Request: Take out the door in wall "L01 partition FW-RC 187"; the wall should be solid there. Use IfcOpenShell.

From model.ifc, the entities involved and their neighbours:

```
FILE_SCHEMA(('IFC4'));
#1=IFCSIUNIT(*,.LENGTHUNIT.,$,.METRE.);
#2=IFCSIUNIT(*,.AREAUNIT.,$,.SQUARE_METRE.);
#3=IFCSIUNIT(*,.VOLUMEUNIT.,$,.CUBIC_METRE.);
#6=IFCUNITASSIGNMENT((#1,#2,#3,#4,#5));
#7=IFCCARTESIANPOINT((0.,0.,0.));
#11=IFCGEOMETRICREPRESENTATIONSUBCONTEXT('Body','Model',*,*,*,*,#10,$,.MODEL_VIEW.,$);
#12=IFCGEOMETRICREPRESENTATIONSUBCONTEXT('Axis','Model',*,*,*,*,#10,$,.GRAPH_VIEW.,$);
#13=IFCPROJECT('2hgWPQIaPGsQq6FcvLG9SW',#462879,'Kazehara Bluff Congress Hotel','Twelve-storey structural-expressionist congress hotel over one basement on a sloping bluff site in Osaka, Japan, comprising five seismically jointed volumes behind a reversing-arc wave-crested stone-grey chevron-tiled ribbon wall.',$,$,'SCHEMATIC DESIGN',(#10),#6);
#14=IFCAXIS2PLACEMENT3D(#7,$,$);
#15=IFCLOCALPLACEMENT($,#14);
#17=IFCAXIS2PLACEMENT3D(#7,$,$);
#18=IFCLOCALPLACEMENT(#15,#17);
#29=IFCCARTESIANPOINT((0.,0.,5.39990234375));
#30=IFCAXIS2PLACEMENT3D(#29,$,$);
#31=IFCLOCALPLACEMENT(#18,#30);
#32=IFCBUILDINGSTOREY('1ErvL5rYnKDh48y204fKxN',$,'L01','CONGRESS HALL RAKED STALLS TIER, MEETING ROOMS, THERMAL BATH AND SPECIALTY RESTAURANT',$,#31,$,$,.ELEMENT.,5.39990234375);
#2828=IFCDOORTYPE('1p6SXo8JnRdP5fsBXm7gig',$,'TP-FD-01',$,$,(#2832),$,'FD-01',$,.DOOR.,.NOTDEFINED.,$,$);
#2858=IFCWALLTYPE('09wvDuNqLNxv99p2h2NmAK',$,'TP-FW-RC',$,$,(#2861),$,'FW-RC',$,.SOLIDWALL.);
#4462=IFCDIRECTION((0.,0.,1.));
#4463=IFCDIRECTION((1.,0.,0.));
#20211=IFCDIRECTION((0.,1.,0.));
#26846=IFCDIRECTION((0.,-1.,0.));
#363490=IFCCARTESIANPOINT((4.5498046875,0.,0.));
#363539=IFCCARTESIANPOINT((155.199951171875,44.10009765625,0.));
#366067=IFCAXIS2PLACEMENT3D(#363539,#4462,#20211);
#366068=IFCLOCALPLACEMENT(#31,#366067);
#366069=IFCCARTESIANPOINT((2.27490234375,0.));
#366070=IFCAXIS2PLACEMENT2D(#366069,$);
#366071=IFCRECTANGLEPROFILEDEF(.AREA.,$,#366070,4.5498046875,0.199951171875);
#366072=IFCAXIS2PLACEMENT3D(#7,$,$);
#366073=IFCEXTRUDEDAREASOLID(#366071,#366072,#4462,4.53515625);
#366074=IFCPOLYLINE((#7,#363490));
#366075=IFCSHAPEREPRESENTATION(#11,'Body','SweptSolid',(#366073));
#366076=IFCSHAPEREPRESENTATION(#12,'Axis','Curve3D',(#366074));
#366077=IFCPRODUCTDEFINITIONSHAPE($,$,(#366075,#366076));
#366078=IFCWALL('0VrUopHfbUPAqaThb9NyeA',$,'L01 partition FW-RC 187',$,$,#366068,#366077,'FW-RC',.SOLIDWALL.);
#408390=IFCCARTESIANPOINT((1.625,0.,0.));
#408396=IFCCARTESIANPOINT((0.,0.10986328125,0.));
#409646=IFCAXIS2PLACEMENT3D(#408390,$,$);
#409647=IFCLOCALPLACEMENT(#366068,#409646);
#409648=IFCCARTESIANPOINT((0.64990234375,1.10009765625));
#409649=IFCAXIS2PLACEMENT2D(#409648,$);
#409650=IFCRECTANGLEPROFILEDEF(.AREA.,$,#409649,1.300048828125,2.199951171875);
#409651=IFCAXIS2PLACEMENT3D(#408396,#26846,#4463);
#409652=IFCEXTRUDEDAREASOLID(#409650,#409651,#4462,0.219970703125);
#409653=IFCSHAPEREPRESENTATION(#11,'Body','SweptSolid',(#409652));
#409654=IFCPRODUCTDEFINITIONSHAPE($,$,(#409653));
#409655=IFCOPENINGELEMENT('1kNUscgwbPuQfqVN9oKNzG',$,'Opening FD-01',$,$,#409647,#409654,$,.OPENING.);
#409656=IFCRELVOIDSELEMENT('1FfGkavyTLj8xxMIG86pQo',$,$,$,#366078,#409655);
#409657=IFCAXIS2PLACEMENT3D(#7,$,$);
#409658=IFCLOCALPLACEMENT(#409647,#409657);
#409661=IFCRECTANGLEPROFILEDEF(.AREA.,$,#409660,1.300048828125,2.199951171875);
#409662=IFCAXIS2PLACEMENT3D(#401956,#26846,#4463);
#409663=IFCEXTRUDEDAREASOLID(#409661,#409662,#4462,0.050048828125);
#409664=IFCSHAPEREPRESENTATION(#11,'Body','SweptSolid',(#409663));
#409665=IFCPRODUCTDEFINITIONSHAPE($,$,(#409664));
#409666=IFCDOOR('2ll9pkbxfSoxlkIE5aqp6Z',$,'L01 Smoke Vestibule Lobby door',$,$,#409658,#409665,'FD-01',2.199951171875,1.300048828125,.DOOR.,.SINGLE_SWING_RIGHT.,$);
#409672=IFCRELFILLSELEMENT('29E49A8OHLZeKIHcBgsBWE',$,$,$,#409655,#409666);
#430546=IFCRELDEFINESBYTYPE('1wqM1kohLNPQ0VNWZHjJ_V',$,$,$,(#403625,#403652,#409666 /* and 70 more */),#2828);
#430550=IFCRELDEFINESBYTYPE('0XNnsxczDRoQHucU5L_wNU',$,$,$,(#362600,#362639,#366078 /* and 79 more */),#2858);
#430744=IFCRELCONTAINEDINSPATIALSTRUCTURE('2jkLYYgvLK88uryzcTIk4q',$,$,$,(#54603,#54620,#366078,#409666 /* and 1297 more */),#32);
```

```python
import ifcopenshell
import ifcopenshell.api.feature
import ifcopenshell.api.root
import ifcopenshell.geom
import ifcopenshell.util.shape

model = ifcopenshell.open("model.ifc")
settings = ifcopenshell.geom.settings()


def volume(element):
    """Net volume in cubic metres, openings subtracted."""
    shape = ifcopenshell.geom.create_shape(settings, element)
    return ifcopenshell.util.shape.get_volume(shape.geometry)


door = model.by_guid("2ll9pkbxfSoxlkIE5aqp6Z")
opening = door.FillsVoids[0].RelatingOpeningElement
wall = opening.VoidsElements[0].RelatingBuildingElement
before = volume(wall)

ifcopenshell.api.root.remove_product(model, product=door)
ifcopenshell.api.feature.remove_feature(model, feature=opening)

after = volume(wall)

print(f"wall volume {before:.3f} -> {after:.3f} m3")

model.write("model_updated.ifc")
```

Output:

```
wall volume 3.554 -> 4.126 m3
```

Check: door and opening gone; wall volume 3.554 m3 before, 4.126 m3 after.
